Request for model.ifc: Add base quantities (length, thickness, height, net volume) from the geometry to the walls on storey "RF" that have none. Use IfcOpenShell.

First a look at what the model holds.

```python
import ifcopenshell
import ifcopenshell.util.element
import ifcopenshell.util.unit

model = ifcopenshell.open("model.ifc")
print(model.schema)
for unit_type in ("LENGTHUNIT", "AREAUNIT", "VOLUMEUNIT"):
    print(unit_type, ifcopenshell.util.unit.calculate_unit_scale(model, unit_type))
storey = next(s for s in model.by_type("IfcBuildingStorey") if s.Name == "RF")
walls = [e for e in ifcopenshell.util.element.get_decomposition(storey) if e.is_a("IfcWall")]
for e in sorted(walls, key=lambda e: e.id()):
    print(e.id(), e.is_a(), e.Name, list(ifcopenshell.util.element.get_psets(e, qtos_only=True)), sep=" | ")
```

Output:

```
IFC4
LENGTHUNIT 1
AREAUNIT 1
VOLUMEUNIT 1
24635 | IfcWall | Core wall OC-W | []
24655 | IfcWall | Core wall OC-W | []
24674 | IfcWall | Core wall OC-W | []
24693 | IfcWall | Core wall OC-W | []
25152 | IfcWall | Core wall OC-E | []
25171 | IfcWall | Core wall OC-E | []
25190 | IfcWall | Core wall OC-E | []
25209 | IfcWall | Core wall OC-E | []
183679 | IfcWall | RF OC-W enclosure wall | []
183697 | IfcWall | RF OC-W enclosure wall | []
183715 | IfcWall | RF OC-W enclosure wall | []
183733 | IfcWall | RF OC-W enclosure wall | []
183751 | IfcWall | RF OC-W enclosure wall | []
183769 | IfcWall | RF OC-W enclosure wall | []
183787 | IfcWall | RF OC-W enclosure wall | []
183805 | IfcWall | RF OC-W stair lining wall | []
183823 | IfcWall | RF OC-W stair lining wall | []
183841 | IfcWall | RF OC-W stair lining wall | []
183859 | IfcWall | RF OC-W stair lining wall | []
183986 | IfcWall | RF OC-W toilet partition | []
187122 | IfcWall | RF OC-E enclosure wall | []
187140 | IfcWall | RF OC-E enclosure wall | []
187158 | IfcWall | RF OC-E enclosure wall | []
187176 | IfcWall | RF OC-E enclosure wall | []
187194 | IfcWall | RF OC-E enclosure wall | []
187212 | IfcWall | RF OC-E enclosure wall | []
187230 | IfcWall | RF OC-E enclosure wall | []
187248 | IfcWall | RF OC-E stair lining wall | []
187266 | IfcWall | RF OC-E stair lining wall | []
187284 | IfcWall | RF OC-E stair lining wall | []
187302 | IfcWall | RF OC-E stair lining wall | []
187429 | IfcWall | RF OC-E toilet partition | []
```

```python
import ifcopenshell
import ifcopenshell.api.pset
import ifcopenshell.geom
import ifcopenshell.util.element
import ifcopenshell.util.shape
import ifcopenshell.util.unit

model = ifcopenshell.open("model.ifc")
unit_scale = ifcopenshell.util.unit.calculate_unit_scale(model)
volume_scale = ifcopenshell.util.unit.calculate_unit_scale(model, "VOLUMEUNIT")
settings = ifcopenshell.geom.settings()

storey = next(s for s in model.by_type("IfcBuildingStorey") if s.Name == "RF")
walls = [e for e in ifcopenshell.util.element.get_decomposition(storey) if e.is_a("IfcWall")]

for e in sorted(walls, key=lambda e: e.id()):
    if ifcopenshell.util.element.get_psets(e, qtos_only=True, should_inherit=False):
        continue
    # Geometry comes back in metres, in the element's own axes.
    shape = ifcopenshell.geom.create_shape(settings, e)
    values = {
        "Length": ifcopenshell.util.shape.get_x(shape.geometry) / unit_scale,
        "Width": ifcopenshell.util.shape.get_y(shape.geometry) / unit_scale,
        "Height": ifcopenshell.util.shape.get_z(shape.geometry) / unit_scale,
        "NetVolume": ifcopenshell.util.shape.get_volume(shape.geometry) / volume_scale,
    }
    qto = ifcopenshell.api.pset.add_qto(model, product=e, name="Qto_WallBaseQuantities")
    ifcopenshell.api.pset.edit_qto(model, qto=qto, properties=values)
    print(e.id(), {k: round(v, 3) for k, v in values.items()})

model.write("model_rev.ifc")
```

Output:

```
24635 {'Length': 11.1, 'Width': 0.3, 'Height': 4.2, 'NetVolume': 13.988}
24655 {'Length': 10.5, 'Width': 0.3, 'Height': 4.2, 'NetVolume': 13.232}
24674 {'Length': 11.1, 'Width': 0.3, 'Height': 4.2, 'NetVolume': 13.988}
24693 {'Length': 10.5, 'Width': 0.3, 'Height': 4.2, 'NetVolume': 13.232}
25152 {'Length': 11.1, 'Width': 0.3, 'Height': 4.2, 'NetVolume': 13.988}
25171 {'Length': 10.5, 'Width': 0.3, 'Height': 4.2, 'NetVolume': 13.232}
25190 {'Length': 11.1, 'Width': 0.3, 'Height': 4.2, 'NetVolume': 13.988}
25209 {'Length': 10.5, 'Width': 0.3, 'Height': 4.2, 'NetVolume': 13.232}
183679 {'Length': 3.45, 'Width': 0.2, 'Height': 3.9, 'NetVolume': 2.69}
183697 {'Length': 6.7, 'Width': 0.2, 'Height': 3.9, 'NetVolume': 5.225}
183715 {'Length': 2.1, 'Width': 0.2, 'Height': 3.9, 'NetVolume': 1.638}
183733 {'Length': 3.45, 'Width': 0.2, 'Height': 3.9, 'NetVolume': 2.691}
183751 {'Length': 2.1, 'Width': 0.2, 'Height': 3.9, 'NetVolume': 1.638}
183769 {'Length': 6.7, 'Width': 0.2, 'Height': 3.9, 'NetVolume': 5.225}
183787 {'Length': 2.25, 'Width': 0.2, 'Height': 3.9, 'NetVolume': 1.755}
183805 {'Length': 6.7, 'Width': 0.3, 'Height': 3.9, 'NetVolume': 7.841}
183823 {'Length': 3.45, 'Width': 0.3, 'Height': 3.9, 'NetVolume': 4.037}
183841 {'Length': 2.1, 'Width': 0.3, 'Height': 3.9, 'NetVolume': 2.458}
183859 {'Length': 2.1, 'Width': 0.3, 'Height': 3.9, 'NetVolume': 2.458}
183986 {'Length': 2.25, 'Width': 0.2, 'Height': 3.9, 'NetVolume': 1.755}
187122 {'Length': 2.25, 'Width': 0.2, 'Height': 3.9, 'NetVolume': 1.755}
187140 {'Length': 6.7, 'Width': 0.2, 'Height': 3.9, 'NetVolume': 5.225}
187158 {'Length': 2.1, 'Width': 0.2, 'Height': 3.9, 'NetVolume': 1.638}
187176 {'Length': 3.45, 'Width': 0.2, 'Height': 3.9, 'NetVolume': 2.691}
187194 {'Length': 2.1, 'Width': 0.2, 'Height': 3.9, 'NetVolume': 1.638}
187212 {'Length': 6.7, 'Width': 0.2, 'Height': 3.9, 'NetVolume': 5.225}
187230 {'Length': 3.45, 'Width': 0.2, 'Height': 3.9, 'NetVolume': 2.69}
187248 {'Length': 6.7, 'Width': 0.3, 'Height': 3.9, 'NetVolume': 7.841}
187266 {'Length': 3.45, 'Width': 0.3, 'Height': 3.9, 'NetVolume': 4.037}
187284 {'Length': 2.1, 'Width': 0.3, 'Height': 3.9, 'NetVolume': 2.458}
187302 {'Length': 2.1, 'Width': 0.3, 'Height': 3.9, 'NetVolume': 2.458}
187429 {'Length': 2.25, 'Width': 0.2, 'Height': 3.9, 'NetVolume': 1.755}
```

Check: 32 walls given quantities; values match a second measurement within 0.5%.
